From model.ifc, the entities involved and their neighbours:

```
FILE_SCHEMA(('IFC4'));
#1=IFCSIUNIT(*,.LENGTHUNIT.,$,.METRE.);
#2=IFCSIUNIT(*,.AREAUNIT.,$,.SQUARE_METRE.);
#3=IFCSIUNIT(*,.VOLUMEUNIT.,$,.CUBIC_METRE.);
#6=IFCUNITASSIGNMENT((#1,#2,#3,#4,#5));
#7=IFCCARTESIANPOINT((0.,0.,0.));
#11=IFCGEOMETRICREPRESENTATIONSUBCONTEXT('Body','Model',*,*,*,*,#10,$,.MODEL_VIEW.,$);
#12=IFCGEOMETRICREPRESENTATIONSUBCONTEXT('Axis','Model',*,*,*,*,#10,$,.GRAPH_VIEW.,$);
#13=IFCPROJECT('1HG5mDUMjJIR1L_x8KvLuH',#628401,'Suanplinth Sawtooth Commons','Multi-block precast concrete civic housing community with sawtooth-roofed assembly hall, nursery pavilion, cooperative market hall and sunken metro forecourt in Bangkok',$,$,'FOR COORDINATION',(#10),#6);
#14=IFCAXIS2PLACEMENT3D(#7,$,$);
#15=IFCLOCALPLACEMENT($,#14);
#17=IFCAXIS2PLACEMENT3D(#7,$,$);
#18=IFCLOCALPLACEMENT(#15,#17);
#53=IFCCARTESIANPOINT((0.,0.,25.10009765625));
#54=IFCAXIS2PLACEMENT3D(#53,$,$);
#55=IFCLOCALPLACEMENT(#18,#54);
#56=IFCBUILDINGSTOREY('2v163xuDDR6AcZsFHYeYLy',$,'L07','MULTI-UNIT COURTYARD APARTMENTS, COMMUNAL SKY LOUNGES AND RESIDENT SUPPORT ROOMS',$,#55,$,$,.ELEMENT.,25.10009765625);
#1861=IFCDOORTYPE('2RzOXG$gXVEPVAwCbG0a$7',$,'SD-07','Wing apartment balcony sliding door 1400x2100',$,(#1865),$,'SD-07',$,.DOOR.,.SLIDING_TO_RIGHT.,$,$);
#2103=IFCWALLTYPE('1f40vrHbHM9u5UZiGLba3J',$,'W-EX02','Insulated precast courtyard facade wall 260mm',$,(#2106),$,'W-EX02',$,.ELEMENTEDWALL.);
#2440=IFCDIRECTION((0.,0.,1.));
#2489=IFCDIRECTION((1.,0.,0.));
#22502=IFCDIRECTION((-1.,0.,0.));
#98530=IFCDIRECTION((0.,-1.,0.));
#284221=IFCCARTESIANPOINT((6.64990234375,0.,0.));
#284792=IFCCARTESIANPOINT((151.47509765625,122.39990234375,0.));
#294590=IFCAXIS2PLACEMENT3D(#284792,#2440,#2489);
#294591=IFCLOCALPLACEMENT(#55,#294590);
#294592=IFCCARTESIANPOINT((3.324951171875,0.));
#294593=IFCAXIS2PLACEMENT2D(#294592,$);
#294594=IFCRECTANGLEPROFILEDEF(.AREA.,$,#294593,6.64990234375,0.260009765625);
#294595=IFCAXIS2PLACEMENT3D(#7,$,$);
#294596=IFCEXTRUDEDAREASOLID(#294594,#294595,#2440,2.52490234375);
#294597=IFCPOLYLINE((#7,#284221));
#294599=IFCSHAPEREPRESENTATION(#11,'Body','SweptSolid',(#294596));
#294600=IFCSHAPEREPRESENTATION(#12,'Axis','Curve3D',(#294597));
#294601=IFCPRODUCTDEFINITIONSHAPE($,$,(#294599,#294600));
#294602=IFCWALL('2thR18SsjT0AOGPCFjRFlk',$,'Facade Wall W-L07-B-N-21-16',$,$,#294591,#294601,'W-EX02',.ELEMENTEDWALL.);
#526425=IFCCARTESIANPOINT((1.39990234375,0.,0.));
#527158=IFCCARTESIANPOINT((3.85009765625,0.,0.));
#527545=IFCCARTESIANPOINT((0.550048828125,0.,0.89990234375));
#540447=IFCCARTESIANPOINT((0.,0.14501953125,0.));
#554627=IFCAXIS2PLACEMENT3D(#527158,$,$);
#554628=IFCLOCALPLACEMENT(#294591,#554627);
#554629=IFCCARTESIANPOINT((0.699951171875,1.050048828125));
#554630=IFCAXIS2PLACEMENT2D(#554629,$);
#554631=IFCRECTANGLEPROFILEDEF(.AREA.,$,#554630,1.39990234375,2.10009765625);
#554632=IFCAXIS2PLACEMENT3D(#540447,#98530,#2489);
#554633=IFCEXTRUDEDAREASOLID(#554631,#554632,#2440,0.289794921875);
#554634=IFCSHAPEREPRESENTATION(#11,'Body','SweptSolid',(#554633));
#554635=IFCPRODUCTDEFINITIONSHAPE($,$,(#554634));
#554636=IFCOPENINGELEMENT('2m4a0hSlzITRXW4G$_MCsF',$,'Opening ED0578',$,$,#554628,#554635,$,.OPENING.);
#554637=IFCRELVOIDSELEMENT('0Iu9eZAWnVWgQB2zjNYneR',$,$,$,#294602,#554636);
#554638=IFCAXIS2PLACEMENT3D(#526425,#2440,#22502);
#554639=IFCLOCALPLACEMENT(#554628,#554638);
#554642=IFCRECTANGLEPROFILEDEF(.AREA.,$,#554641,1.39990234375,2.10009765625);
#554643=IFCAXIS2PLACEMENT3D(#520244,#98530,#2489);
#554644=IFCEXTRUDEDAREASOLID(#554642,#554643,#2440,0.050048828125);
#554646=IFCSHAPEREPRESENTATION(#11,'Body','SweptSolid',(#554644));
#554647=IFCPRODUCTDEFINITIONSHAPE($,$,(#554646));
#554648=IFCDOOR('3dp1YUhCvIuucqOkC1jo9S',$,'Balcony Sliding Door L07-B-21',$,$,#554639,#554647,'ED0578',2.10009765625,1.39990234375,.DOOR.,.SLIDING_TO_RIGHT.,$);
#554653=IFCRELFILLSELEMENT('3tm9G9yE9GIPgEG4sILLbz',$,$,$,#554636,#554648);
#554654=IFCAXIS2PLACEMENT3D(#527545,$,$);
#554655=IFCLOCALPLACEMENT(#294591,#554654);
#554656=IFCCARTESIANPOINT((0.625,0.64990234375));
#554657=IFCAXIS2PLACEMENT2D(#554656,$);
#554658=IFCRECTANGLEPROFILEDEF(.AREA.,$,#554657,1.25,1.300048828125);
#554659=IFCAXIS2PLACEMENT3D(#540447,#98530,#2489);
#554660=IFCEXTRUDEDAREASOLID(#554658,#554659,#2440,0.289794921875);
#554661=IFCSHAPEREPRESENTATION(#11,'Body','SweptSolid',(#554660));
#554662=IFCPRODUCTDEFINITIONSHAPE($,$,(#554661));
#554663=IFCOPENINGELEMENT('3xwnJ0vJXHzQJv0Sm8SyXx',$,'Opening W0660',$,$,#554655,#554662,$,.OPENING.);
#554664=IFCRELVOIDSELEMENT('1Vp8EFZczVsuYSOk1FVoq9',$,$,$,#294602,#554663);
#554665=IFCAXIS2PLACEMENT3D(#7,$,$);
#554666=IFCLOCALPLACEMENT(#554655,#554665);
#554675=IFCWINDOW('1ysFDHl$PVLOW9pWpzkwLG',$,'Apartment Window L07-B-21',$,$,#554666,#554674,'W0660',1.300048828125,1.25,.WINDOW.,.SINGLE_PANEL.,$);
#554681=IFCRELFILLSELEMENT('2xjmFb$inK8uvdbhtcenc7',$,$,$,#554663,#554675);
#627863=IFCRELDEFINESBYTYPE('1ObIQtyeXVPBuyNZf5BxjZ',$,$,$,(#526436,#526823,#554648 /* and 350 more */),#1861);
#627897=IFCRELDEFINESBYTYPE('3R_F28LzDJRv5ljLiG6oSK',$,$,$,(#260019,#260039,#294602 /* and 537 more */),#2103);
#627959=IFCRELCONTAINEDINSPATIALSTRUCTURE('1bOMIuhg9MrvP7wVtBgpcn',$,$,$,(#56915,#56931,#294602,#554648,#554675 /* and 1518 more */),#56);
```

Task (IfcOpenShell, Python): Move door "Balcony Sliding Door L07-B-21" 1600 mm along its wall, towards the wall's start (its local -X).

```python
import ifcopenshell
import ifcopenshell.api.geometry
import ifcopenshell.util.placement
import ifcopenshell.util.unit

model = ifcopenshell.open("model.ifc")
unit_scale = ifcopenshell.util.unit.calculate_unit_scale(model)

door = model.by_guid("3dp1YUhCvIuucqOkC1jo9S")
opening = door.FillsVoids[0].RelatingOpeningElement
wall = opening.VoidsElements[0].RelatingBuildingElement

wall_matrix = ifcopenshell.util.placement.get_local_placement(wall.ObjectPlacement)
shift = wall_matrix[:3, 0] * -1.6 / unit_scale
before = ifcopenshell.util.placement.get_local_placement(door.ObjectPlacement)[:3, 3].copy()

# The door is placed relative to its opening, so it follows when the opening moves.
matrix = ifcopenshell.util.placement.get_local_placement(opening.ObjectPlacement)
matrix[:3, 3] += shift
ifcopenshell.api.geometry.edit_object_placement(
    model, product=opening, matrix=matrix, is_si=False, should_transform_children=True
)

after = ifcopenshell.util.placement.get_local_placement(door.ObjectPlacement)[:3, 3]
print("door moved by", (after - before).round(3) + 0.0)

model.write("model_edited.ifc")
```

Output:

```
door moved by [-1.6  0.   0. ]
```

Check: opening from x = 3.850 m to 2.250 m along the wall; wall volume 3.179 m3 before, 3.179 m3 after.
